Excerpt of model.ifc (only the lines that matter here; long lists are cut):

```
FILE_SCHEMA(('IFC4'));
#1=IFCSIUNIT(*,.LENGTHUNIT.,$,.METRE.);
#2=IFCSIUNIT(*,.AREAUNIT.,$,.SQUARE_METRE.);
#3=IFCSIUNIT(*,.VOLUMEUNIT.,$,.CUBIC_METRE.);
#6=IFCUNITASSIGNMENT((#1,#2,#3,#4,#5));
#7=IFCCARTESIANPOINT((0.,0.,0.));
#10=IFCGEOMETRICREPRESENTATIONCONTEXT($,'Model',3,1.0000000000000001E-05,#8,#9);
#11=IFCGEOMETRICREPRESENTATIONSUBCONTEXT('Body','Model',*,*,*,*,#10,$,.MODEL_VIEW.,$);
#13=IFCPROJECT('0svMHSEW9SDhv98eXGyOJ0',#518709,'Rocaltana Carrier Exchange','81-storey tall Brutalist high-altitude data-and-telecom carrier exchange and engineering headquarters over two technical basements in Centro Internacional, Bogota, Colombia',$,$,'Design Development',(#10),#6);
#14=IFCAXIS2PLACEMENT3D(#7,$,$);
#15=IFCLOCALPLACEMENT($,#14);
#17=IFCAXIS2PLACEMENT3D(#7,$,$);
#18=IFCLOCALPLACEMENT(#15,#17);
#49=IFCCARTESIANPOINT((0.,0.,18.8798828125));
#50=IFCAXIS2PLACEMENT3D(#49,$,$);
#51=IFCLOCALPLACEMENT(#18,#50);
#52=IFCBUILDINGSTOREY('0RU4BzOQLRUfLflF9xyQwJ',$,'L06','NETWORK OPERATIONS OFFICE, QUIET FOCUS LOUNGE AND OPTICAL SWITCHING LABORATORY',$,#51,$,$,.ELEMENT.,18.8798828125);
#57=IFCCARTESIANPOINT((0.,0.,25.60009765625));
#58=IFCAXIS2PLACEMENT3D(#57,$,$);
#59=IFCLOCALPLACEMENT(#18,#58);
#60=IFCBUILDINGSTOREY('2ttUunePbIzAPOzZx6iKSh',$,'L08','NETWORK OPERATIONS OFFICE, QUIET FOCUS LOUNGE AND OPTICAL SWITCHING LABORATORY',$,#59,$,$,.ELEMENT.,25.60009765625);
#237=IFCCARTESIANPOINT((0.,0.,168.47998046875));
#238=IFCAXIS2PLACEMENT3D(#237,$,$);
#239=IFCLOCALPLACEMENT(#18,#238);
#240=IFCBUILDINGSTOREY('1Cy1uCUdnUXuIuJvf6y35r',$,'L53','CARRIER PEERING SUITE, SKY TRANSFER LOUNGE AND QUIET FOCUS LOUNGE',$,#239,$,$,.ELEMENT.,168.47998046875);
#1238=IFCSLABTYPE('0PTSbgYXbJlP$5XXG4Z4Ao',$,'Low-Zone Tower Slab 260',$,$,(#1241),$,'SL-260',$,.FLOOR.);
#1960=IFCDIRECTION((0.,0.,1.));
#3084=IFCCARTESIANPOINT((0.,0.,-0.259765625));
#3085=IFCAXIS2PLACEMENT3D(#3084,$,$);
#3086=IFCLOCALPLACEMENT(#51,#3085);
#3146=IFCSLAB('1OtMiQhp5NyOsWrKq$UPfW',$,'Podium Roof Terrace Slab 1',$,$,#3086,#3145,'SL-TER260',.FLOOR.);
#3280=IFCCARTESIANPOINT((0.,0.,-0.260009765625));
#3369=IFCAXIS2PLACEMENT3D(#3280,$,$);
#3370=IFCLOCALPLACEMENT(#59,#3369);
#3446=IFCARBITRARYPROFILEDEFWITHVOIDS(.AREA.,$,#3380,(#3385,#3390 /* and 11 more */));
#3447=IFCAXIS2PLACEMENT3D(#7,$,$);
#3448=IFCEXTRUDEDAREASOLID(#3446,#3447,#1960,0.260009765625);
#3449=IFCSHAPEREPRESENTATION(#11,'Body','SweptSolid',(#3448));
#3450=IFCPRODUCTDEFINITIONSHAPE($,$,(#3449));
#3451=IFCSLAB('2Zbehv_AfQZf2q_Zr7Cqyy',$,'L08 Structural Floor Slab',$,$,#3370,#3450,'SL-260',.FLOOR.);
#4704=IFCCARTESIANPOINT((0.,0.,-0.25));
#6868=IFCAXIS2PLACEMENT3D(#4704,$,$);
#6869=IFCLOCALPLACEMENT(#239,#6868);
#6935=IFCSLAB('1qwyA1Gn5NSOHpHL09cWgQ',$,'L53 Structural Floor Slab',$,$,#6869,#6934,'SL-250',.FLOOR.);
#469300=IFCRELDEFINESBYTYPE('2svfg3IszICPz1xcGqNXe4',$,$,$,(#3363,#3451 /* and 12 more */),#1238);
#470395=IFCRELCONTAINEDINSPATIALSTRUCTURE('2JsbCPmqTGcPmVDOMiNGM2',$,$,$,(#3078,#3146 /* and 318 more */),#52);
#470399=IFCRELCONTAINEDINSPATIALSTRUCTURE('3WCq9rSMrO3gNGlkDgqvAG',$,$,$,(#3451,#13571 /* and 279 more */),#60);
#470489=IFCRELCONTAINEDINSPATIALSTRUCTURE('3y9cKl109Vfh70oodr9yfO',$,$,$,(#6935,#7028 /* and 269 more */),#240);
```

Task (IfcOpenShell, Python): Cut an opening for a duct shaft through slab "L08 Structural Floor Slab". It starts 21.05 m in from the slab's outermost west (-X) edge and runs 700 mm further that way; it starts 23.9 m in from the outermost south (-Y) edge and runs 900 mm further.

```python
import numpy as np
import ifcopenshell
import ifcopenshell.api.feature
import ifcopenshell.api.geometry
import ifcopenshell.api.root
import ifcopenshell.geom
import ifcopenshell.util.placement
import ifcopenshell.util.representation
import ifcopenshell.util.shape
import ifcopenshell.util.unit

model = ifcopenshell.open("model.ifc")
unit_scale = ifcopenshell.util.unit.calculate_unit_scale(model)
settings = ifcopenshell.geom.settings()


def volume(element):
    """Net volume in cubic metres, openings subtracted."""
    shape = ifcopenshell.geom.create_shape(settings, element)
    return ifcopenshell.util.shape.get_volume(shape.geometry)


slab = model.by_guid("2Zbehv_AfQZf2q_Zr7Cqyy")
before = volume(slab)

# Extent in the slab's own axes, in metres. The edges named are its -X and -Y sides.
slab_shape = ifcopenshell.geom.create_shape(settings, slab)
vertices = ifcopenshell.util.shape.get_vertices(slab_shape.geometry)
x_min, y_min, bottom = vertices.min(axis=0)
top = vertices[:, 2].max()

opening = ifcopenshell.api.root.create_entity(model, ifc_class="IfcOpeningElement", name="Duct shaft opening", predefined_type="OPENING")
context = ifcopenshell.util.representation.get_context(model, "Model", "Body", "MODEL_VIEW")
width, depth = 0.7, 0.9
outline = [(0.0, 0.0), (width, 0.0), (width, depth), (0.0, depth), (0.0, 0.0)]
# Overshoot both faces by 50 mm so the cut is clean.
shape = ifcopenshell.api.geometry.add_slab_representation(
    model, context=context, depth=top - bottom + 0.1, polyline=outline
)
ifcopenshell.api.geometry.assign_representation(model, product=opening, representation=shape)

matrix = ifcopenshell.util.placement.get_local_placement(slab.ObjectPlacement)
matrix[:, 3] = matrix @ np.append(np.array([x_min + 21.05, y_min + 23.9, bottom - 0.05]) / unit_scale, 1.0)
ifcopenshell.api.geometry.edit_object_placement(model, product=opening, matrix=matrix, is_si=False)
ifcopenshell.api.feature.add_feature(model, feature=opening, element=slab)

after = volume(slab)

print(f"slab volume {before:.3f} -> {after:.3f} m3")

model.write("model_rev.ifc")
```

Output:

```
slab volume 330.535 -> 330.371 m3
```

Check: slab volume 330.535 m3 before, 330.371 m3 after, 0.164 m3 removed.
